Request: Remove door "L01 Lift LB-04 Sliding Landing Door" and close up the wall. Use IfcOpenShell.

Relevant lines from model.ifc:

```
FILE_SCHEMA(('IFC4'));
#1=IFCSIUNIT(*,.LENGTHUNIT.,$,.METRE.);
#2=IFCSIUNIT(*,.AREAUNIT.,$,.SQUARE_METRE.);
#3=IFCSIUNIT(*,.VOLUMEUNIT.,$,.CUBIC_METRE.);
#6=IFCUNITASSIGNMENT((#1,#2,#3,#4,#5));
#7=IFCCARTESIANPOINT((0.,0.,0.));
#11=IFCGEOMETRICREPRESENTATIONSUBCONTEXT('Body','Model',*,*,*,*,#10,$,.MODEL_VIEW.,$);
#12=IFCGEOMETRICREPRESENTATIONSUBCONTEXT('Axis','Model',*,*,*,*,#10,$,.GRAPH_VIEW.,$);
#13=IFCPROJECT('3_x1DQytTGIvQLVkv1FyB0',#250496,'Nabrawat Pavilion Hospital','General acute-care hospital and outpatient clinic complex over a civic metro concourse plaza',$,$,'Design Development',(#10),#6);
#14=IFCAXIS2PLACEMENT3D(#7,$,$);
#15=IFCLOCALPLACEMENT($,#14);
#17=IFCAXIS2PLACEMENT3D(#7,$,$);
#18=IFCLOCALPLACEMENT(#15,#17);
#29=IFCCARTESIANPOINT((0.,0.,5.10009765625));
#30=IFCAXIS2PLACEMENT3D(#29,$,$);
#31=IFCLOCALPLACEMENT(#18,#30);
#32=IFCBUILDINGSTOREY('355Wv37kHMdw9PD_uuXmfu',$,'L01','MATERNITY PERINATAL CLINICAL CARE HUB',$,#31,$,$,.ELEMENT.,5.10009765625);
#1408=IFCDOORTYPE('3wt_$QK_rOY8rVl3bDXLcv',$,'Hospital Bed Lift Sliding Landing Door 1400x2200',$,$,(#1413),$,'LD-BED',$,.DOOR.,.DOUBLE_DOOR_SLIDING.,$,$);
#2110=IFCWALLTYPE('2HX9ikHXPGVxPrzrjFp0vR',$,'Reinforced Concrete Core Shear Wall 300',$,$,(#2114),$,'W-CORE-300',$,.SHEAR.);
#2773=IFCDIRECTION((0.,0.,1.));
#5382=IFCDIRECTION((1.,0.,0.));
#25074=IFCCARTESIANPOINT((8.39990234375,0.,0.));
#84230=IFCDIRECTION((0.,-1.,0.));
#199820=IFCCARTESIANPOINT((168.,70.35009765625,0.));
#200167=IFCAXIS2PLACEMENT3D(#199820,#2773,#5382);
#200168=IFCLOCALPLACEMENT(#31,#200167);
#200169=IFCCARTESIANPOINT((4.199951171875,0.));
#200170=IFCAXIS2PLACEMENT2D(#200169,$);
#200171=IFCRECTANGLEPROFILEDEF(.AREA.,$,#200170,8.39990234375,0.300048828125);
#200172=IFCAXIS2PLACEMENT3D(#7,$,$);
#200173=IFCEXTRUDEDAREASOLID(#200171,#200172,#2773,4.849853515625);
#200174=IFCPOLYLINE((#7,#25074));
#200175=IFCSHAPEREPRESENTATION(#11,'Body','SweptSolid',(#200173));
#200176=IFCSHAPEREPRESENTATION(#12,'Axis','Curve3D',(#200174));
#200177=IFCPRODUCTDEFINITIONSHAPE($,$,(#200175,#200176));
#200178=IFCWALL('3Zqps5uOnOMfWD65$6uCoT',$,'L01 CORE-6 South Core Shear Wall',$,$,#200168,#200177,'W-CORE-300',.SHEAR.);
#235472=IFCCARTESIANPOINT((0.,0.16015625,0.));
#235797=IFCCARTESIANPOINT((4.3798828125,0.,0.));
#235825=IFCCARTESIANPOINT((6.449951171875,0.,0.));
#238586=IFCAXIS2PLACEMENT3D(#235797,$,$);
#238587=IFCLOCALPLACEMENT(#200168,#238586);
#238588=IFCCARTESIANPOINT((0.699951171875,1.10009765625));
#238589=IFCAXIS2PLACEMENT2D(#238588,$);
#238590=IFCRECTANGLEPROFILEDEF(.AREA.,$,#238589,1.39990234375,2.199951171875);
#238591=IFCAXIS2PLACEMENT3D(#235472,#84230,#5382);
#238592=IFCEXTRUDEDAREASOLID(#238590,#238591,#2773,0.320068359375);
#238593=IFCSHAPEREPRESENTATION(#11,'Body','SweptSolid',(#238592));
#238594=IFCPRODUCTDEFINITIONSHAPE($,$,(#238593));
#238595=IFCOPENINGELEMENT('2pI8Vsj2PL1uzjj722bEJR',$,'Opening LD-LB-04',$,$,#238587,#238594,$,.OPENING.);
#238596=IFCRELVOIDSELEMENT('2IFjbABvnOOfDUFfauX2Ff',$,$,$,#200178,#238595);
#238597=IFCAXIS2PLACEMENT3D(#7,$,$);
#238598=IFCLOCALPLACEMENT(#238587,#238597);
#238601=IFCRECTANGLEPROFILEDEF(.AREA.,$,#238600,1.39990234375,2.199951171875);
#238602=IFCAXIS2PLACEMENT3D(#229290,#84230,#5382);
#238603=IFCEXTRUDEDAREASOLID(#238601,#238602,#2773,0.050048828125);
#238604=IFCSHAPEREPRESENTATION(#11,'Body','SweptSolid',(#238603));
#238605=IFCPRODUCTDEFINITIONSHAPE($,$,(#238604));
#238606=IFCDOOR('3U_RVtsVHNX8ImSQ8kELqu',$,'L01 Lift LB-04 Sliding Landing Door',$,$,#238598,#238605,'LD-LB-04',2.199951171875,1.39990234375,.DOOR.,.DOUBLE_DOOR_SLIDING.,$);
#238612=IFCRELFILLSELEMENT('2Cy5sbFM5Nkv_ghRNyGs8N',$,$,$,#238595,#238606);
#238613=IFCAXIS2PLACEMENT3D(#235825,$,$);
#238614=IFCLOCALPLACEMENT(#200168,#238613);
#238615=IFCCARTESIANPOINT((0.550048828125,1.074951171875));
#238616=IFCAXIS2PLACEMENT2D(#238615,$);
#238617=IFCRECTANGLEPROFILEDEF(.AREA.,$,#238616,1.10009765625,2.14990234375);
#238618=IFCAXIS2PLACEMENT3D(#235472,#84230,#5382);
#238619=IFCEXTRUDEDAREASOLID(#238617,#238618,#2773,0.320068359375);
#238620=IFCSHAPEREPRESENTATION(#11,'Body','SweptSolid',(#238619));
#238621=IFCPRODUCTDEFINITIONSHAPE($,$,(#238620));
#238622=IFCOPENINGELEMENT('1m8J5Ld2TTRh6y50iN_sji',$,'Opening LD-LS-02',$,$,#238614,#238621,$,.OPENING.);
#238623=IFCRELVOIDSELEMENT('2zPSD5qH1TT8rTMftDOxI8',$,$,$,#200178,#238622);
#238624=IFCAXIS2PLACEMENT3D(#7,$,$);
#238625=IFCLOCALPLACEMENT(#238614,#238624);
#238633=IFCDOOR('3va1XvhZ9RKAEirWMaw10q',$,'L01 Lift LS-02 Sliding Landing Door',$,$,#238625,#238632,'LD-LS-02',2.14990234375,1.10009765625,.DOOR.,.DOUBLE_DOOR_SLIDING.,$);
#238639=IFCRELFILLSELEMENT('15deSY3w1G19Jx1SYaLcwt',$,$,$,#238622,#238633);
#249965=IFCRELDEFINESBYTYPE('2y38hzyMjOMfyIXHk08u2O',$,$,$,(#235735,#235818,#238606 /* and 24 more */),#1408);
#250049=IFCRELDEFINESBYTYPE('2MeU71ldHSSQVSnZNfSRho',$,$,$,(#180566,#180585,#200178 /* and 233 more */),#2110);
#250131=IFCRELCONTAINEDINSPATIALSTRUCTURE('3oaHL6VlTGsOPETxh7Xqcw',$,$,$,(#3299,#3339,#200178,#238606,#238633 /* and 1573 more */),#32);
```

```python
import ifcopenshell
import ifcopenshell.api.feature
import ifcopenshell.api.root
import ifcopenshell.geom
import ifcopenshell.util.shape

model = ifcopenshell.open("model.ifc")
settings = ifcopenshell.geom.settings()


def volume(element):
    """Net volume in cubic metres, openings subtracted."""
    shape = ifcopenshell.geom.create_shape(settings, element)
    return ifcopenshell.util.shape.get_volume(shape.geometry)


door = model.by_id(238606)
opening = door.FillsVoids[0].RelatingOpeningElement
wall = opening.VoidsElements[0].RelatingBuildingElement
before = volume(wall)

ifcopenshell.api.root.remove_product(model, product=door)
ifcopenshell.api.feature.remove_feature(model, feature=opening)

after = volume(wall)

print(f"wall volume {before:.3f} -> {after:.3f} m3")

model.write("model_edited.ifc")
```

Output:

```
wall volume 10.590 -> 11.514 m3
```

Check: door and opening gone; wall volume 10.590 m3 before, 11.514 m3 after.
